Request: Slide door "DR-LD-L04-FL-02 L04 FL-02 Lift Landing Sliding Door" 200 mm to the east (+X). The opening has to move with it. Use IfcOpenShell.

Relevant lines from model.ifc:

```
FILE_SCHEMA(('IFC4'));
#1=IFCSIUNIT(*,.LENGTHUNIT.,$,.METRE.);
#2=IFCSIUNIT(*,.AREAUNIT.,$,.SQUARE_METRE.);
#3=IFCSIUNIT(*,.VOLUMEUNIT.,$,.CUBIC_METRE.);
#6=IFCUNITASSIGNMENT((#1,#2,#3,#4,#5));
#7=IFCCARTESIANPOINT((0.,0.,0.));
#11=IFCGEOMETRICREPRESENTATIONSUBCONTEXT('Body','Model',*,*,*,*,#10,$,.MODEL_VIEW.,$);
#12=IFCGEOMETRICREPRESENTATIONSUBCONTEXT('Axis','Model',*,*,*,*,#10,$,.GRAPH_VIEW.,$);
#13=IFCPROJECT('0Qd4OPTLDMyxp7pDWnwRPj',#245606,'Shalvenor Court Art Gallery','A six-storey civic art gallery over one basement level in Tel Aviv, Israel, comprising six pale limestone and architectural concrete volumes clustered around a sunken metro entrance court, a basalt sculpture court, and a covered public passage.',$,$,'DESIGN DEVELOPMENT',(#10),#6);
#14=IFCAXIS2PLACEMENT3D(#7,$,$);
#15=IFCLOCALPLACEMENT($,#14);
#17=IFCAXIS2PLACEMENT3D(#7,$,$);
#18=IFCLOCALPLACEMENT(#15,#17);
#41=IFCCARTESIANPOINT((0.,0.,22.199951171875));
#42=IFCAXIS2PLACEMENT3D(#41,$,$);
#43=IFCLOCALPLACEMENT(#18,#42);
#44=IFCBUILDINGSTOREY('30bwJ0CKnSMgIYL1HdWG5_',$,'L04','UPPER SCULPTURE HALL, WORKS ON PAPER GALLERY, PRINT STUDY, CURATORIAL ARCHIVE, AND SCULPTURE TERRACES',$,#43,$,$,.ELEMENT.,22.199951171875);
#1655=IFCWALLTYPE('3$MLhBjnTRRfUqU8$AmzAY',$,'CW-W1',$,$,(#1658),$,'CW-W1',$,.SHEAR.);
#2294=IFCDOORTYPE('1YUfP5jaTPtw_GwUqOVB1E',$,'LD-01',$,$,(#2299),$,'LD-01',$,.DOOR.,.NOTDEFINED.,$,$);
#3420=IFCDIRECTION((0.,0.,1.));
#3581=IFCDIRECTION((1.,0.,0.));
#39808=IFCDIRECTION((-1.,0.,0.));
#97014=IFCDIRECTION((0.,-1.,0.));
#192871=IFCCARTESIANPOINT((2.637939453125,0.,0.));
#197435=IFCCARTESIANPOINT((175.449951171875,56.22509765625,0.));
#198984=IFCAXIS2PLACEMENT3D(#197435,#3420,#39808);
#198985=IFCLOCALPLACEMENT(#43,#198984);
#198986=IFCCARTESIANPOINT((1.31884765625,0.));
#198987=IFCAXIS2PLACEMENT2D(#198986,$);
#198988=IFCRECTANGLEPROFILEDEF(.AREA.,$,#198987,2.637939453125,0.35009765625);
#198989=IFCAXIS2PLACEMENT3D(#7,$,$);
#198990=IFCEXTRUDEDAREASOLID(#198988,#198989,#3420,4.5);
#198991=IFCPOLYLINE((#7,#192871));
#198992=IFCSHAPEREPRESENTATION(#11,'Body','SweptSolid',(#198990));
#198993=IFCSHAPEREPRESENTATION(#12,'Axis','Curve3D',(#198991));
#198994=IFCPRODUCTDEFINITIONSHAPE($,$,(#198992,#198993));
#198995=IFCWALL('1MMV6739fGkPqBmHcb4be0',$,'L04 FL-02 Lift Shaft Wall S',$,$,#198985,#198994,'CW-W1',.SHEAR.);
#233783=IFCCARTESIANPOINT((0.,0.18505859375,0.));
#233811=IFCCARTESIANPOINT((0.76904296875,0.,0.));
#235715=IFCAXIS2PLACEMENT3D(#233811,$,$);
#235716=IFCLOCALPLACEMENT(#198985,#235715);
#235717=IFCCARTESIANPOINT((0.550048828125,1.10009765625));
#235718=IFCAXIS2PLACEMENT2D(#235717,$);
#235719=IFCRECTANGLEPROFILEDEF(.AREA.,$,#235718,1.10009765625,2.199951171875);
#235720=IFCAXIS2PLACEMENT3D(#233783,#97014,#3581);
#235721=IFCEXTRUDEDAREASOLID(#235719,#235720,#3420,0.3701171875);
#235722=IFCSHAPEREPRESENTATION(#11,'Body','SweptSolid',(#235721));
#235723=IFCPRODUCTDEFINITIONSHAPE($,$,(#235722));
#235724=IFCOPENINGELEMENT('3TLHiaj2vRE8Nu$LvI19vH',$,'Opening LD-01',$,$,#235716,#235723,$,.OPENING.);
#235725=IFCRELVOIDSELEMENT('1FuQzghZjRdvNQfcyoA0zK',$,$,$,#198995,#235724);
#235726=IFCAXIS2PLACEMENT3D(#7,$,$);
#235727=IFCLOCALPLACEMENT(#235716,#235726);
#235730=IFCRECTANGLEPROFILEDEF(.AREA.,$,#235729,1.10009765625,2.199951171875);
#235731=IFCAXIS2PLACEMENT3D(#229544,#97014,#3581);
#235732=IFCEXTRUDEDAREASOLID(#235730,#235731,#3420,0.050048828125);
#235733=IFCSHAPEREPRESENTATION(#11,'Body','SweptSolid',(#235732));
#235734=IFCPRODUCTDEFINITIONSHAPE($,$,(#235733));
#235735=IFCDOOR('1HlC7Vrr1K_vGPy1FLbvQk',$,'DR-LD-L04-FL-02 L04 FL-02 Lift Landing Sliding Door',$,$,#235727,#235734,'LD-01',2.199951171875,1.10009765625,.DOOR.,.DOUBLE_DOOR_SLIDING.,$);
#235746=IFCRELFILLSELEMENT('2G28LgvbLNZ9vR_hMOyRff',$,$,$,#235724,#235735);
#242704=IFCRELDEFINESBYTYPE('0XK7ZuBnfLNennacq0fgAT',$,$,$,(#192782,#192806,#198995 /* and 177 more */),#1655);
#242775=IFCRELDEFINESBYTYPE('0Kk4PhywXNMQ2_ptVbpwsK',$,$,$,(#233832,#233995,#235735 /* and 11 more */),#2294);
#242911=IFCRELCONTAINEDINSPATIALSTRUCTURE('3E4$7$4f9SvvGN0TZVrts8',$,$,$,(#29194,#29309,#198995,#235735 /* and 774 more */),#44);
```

```python
import ifcopenshell
import ifcopenshell.api.geometry
import ifcopenshell.util.placement
import ifcopenshell.util.unit

model = ifcopenshell.open("model.ifc")
unit_scale = ifcopenshell.util.unit.calculate_unit_scale(model)

door = model.by_guid("1HlC7Vrr1K_vGPy1FLbvQk")
opening = door.FillsVoids[0].RelatingOpeningElement
wall = opening.VoidsElements[0].RelatingBuildingElement

wall_matrix = ifcopenshell.util.placement.get_local_placement(wall.ObjectPlacement)
shift = wall_matrix[:3, 0] * -0.2 / unit_scale
before = ifcopenshell.util.placement.get_local_placement(door.ObjectPlacement)[:3, 3].copy()

# The door is placed relative to its opening, so it follows when the opening moves.
matrix = ifcopenshell.util.placement.get_local_placement(opening.ObjectPlacement)
matrix[:3, 3] += shift
ifcopenshell.api.geometry.edit_object_placement(
    model, product=opening, matrix=matrix, is_si=False, should_transform_children=True
)

after = ifcopenshell.util.placement.get_local_placement(door.ObjectPlacement)[:3, 3]
print("door moved by", (after - before).round(3) + 0.0)

model.write("model_v2.ifc")
```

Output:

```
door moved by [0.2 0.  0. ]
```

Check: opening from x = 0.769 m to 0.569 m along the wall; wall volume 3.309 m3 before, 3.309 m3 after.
